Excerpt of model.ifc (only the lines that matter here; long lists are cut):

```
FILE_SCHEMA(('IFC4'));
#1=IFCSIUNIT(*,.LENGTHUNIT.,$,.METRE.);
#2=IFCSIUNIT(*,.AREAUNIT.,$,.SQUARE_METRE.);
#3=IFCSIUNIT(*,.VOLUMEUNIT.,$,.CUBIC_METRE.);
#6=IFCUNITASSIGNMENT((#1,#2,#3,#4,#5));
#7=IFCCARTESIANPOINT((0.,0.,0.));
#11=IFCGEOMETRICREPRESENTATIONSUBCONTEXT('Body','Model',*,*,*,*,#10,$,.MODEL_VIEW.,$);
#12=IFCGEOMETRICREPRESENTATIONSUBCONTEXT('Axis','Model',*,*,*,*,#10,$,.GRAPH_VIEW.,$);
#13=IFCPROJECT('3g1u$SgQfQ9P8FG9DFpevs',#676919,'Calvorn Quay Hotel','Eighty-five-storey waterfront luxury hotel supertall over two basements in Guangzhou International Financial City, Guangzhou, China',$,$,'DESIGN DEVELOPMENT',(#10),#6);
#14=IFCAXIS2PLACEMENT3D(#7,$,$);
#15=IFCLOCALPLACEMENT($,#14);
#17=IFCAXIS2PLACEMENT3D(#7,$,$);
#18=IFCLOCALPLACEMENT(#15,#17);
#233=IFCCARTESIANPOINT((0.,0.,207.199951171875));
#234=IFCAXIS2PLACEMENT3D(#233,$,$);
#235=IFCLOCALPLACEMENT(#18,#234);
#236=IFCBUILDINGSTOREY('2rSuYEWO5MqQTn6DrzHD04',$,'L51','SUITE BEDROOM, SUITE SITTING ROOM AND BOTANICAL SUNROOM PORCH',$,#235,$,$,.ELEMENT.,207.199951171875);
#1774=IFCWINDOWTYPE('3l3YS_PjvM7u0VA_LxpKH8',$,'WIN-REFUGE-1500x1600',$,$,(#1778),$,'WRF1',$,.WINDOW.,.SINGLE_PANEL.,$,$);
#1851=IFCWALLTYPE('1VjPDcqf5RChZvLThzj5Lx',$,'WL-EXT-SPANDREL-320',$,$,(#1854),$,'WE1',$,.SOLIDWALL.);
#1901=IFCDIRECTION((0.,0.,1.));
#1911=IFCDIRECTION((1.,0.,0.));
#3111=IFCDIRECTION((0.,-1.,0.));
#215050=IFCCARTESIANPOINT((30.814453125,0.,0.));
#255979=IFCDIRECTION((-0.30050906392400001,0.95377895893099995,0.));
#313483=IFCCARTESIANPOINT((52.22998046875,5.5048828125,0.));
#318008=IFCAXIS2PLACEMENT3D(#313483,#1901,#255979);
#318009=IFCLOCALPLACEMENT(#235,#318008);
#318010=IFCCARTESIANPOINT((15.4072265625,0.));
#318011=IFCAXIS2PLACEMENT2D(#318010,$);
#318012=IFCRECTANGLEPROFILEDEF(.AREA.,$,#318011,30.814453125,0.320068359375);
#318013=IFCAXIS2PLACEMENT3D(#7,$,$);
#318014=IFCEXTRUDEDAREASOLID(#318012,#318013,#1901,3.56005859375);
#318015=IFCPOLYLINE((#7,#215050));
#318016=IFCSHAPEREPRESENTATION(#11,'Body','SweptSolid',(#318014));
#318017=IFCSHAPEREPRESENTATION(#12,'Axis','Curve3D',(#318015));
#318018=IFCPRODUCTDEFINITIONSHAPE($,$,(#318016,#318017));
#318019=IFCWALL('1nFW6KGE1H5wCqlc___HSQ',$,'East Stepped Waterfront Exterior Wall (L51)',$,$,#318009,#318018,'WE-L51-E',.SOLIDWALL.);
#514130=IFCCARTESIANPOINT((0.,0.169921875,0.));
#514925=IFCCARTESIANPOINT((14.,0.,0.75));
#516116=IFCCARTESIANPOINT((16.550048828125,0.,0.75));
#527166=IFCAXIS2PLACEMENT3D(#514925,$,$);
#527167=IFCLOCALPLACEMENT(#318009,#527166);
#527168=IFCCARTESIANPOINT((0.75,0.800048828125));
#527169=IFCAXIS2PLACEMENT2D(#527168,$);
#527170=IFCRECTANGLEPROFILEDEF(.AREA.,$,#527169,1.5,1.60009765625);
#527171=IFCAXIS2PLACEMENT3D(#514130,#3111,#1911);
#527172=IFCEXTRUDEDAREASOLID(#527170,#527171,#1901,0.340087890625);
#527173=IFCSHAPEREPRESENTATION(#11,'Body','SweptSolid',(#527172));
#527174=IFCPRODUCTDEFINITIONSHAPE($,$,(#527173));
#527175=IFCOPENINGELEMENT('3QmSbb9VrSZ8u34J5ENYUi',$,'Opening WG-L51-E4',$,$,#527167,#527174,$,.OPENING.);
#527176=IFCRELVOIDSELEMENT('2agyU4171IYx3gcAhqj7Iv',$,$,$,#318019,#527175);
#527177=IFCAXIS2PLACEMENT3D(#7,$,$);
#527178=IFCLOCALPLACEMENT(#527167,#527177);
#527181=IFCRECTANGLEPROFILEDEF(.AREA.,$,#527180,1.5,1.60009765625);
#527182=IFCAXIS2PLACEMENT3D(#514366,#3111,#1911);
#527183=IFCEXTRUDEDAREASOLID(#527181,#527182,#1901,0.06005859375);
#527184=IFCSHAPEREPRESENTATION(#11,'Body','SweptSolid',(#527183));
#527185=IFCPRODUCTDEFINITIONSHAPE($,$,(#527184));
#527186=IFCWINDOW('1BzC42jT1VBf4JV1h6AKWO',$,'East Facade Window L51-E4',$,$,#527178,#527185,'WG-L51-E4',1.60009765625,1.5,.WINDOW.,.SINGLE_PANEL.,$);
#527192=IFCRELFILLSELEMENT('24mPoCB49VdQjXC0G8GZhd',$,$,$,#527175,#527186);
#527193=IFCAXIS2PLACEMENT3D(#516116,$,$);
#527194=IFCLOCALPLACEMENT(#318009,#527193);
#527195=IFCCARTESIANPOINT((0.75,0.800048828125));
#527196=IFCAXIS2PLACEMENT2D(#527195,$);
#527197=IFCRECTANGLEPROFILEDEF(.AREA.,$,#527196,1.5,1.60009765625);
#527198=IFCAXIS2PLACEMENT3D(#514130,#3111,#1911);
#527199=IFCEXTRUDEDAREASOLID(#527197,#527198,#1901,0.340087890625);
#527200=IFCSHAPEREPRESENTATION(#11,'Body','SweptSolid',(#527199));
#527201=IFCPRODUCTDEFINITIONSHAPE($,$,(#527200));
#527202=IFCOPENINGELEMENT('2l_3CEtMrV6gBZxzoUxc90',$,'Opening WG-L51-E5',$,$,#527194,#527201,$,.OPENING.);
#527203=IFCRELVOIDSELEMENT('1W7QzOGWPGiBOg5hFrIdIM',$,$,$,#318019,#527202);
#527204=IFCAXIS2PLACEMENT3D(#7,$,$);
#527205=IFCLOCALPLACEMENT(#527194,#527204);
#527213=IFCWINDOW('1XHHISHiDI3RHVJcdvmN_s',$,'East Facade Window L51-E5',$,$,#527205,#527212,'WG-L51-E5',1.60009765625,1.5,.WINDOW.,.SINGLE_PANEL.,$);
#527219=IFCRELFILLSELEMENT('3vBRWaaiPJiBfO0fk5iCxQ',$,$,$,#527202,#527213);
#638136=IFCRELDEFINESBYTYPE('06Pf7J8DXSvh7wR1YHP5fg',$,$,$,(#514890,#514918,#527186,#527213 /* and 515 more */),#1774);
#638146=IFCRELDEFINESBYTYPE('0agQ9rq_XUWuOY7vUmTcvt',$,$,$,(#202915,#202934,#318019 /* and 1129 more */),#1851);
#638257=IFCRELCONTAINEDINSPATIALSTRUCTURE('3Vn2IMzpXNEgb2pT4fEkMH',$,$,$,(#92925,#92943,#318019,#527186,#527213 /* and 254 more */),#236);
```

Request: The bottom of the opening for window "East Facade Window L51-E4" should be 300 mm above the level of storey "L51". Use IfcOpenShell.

```python
import numpy as np
import ifcopenshell
import ifcopenshell.api.geometry
import ifcopenshell.geom
import ifcopenshell.util.element
import ifcopenshell.util.placement
import ifcopenshell.util.shape
import ifcopenshell.util.unit

model = ifcopenshell.open("model.ifc")
unit_scale = ifcopenshell.util.unit.calculate_unit_scale(model)

window = model.by_id(527186)
opening = window.FillsVoids[0].RelatingOpeningElement
storey = ifcopenshell.util.element.get_container(window, ifc_class="IfcBuildingStorey")
level = ifcopenshell.util.placement.get_local_placement(storey.ObjectPlacement)[2, 3]

# The opening's origin need not be at the sill, so measure its lowest point.
shape = ifcopenshell.geom.create_shape(ifcopenshell.geom.settings(), opening)
bottom = ifcopenshell.util.shape.get_shape_bottom_elevation(shape, shape.geometry) / unit_scale
dz = level + 0.3 / unit_scale - bottom

shift = np.array([0.0, 0.0, dz])
# The window is placed relative to its opening, so it follows when the opening moves.
matrix = ifcopenshell.util.placement.get_local_placement(opening.ObjectPlacement)
matrix[:3, 3] += shift
ifcopenshell.api.geometry.edit_object_placement(
    model, product=opening, matrix=matrix, is_si=False, should_transform_children=True
)

print(f"moved by {dz * unit_scale:+.3f} m")

model.write("model_rev.ifc")
```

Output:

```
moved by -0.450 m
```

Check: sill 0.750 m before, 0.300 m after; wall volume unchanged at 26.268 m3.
